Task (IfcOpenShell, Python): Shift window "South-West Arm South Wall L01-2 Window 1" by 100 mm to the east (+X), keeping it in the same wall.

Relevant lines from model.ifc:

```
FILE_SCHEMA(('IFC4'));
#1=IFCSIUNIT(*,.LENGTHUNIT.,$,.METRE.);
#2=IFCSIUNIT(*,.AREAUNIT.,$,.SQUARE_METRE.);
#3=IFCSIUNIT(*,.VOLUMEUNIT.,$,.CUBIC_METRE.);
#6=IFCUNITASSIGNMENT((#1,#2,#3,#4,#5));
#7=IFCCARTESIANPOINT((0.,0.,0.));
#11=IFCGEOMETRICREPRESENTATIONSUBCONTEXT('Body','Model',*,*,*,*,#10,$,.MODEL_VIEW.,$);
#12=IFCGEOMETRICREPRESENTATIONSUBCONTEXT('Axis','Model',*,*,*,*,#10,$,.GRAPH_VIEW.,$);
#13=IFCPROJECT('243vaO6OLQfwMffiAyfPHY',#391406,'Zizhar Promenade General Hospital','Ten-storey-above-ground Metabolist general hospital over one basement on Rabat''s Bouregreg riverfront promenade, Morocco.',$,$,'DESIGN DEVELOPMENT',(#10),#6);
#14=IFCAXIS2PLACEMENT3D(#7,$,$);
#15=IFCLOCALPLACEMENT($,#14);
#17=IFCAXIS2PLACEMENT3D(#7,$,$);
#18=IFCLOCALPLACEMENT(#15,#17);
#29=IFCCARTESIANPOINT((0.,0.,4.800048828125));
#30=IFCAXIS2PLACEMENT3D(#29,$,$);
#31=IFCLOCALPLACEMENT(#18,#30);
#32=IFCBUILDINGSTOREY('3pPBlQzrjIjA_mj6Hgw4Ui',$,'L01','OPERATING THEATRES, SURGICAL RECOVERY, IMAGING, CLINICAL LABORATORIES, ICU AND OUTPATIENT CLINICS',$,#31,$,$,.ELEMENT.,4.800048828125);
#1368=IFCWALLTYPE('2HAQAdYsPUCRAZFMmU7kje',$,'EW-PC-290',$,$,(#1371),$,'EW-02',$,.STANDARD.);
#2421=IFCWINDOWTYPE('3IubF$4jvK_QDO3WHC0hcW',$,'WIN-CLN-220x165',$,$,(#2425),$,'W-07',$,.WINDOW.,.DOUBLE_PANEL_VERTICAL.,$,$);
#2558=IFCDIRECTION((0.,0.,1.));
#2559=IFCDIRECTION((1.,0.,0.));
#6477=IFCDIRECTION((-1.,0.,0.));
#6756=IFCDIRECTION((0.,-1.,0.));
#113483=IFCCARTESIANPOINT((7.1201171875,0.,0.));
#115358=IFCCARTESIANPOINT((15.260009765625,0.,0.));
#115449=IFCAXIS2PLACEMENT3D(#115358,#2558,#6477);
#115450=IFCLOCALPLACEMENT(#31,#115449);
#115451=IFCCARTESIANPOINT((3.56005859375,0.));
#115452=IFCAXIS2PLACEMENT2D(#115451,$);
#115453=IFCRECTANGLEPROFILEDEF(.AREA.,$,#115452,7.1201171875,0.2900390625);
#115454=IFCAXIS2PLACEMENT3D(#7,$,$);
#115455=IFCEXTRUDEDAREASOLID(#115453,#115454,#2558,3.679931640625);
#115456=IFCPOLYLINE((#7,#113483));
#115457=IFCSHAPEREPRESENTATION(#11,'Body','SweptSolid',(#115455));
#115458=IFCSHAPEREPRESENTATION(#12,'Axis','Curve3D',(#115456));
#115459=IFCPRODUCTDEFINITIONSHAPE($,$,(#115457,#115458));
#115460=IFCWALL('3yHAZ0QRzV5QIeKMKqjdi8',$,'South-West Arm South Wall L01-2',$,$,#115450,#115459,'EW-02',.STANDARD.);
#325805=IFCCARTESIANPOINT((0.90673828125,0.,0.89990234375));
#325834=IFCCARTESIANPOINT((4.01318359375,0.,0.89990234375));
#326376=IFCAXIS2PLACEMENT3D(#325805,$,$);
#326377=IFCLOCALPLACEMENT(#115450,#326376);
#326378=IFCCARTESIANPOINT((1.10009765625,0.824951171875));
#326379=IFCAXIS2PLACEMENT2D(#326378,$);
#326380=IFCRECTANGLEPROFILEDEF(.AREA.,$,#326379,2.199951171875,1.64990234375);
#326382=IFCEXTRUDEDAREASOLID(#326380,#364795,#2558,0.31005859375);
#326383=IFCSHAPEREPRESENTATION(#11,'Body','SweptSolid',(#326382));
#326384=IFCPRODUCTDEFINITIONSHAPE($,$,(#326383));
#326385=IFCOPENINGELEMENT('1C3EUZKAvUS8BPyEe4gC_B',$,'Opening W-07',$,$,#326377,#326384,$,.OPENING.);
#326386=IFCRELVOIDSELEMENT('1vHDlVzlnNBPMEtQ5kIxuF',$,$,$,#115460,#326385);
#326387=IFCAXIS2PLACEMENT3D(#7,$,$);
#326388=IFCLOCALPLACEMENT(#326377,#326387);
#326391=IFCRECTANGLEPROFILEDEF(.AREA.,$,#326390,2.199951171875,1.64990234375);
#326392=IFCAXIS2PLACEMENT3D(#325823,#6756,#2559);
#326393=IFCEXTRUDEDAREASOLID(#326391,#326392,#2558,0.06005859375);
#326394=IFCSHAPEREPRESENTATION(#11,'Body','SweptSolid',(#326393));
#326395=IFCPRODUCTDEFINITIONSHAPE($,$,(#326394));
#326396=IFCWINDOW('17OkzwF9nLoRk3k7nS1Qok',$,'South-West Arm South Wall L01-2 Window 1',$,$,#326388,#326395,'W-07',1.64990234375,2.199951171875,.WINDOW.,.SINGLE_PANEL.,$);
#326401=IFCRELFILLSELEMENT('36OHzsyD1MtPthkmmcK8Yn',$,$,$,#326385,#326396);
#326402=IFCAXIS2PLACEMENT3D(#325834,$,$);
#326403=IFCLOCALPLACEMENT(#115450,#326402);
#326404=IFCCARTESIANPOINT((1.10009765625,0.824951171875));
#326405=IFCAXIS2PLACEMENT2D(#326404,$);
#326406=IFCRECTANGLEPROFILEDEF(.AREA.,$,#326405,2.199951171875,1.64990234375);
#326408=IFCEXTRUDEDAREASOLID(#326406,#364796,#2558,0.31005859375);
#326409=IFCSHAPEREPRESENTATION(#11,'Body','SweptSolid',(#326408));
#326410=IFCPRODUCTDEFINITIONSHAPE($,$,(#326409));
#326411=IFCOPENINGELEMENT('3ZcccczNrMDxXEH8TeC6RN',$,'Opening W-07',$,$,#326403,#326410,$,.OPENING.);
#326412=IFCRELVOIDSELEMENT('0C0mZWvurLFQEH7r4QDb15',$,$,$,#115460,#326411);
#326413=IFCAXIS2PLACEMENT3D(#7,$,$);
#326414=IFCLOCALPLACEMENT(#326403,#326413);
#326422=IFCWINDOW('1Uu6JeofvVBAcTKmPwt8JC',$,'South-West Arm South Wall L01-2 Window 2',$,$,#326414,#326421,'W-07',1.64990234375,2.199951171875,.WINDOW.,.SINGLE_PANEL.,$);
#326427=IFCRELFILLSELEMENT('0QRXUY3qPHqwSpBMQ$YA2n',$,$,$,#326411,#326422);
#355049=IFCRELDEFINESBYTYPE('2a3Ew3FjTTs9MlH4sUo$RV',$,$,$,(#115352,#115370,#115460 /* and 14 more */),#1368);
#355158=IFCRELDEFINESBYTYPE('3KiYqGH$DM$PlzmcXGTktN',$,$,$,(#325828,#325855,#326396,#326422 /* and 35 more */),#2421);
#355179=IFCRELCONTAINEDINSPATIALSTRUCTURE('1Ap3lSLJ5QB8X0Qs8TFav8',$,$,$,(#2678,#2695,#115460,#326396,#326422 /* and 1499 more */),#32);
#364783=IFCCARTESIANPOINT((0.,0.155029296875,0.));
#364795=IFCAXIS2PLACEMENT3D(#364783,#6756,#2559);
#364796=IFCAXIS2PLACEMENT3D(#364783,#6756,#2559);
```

```python
import ifcopenshell
import ifcopenshell.api.geometry
import ifcopenshell.util.placement

model = ifcopenshell.open("model.ifc")

window = model.by_guid("17OkzwF9nLoRk3k7nS1Qok")
opening = window.FillsVoids[0].RelatingOpeningElement
wall = opening.VoidsElements[0].RelatingBuildingElement

wall_matrix = ifcopenshell.util.placement.get_local_placement(wall.ObjectPlacement)
shift = wall_matrix[:3, 0] * -0.1
before = ifcopenshell.util.placement.get_local_placement(window.ObjectPlacement)[:3, 3].copy()

# The window is placed relative to its opening, so it follows when the opening moves.
matrix = ifcopenshell.util.placement.get_local_placement(opening.ObjectPlacement)
matrix[:3, 3] += shift
ifcopenshell.api.geometry.edit_object_placement(
    model, product=opening, matrix=matrix, is_si=False, should_transform_children=True
)

after = ifcopenshell.util.placement.get_local_placement(window.ObjectPlacement)[:3, 3]
print("window moved by", (after - before).round(3) + 0.0)

model.write("model-out.ifc")
```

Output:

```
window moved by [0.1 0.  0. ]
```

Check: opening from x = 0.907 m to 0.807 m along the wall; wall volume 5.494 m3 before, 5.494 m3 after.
